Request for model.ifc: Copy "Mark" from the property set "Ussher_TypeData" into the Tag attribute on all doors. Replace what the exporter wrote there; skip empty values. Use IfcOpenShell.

First a look at what the model holds.

```python
import ifcopenshell
import ifcopenshell.util.element

model = ifcopenshell.open("model.ifc")
print(model.schema)
doors = model.by_type("IfcDoor")
print(len(doors), "doors")
for e in doors[:8]:
    source = ifcopenshell.util.element.get_pset(e, "Ussher_TypeData", "Mark")
    target = e.Tag
    print(e.id(), repr(source), repr(target), sep=" | ")
```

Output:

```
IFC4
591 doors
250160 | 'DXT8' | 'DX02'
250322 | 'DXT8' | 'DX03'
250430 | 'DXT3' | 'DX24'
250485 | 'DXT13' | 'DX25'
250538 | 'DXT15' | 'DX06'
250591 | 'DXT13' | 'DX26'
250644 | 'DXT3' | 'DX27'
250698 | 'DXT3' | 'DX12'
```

```python
import ifcopenshell
import ifcopenshell.util.element

model = ifcopenshell.open("model.ifc")

count = 0
for e in model.by_type("IfcDoor"):
    value = ifcopenshell.util.element.get_pset(e, "Ussher_TypeData", "Mark")
    current = e.Tag
    if not value or not value.strip() or current == value:
        continue
    e.Tag = value
    count += 1

print(count, "doors updated")

model.write("model_v2.ifc")
```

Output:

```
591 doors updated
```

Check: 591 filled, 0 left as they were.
